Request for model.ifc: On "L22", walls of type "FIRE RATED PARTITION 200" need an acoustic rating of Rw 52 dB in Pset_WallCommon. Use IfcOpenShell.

First a look at what the model holds.

```python
import ifcopenshell
import ifcopenshell.util.element

model = ifcopenshell.open("model.ifc")
print(model.schema)
storey = next(s for s in model.by_type("IfcBuildingStorey") if s.Name == "L22")
walls = [e for e in ifcopenshell.util.element.get_decomposition(storey) if e.is_a("IfcWall")]
seen = {}
for e in walls:
    element_type = ifcopenshell.util.element.get_type(e)
    key = (element_type.Name if element_type != e and element_type else None, ifcopenshell.util.element.get_pset(e, "Pset_WallCommon", "AcousticRating"))
    seen[key] = seen.get(key, 0) + 1
for (name, value), count in sorted(seen.items(), key=str):
    print(count, "x", name, "|", value)
```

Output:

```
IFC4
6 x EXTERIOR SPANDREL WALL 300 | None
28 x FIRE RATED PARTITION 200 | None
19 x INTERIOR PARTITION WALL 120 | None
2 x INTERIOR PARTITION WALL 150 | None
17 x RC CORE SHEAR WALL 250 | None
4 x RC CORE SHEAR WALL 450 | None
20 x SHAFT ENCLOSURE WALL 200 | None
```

```python
import ifcopenshell
import ifcopenshell.api.pset
import ifcopenshell.util.element

model = ifcopenshell.open("model.ifc")

storey = next(s for s in model.by_type("IfcBuildingStorey") if s.Name == "L22")
walls = [e for e in ifcopenshell.util.element.get_decomposition(storey) if e.is_a("IfcWall")]

count = 0
for e in walls:
    element_type = ifcopenshell.util.element.get_type(e)
    if element_type in (None, e) or element_type.Name != "FIRE RATED PARTITION 200":
        continue
    found = ifcopenshell.util.element.get_pset(e, "Pset_WallCommon", should_inherit=False)
    if found:
        pset = model.by_id(found["id"])
        if len(ifcopenshell.util.element.get_elements_by_pset(pset)) > 1:
            pset = ifcopenshell.api.pset.unshare_pset(model, products=[e], pset=pset)[0]
    else:
        pset = ifcopenshell.api.pset.add_pset(model, product=e, name="Pset_WallCommon")
    ifcopenshell.api.pset.edit_pset(model, pset=pset, properties={"AcousticRating": "Rw 52 dB"})
    count += 1

print(count, "walls updated")

model.write("model_rev.ifc")
```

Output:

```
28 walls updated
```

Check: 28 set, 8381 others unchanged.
